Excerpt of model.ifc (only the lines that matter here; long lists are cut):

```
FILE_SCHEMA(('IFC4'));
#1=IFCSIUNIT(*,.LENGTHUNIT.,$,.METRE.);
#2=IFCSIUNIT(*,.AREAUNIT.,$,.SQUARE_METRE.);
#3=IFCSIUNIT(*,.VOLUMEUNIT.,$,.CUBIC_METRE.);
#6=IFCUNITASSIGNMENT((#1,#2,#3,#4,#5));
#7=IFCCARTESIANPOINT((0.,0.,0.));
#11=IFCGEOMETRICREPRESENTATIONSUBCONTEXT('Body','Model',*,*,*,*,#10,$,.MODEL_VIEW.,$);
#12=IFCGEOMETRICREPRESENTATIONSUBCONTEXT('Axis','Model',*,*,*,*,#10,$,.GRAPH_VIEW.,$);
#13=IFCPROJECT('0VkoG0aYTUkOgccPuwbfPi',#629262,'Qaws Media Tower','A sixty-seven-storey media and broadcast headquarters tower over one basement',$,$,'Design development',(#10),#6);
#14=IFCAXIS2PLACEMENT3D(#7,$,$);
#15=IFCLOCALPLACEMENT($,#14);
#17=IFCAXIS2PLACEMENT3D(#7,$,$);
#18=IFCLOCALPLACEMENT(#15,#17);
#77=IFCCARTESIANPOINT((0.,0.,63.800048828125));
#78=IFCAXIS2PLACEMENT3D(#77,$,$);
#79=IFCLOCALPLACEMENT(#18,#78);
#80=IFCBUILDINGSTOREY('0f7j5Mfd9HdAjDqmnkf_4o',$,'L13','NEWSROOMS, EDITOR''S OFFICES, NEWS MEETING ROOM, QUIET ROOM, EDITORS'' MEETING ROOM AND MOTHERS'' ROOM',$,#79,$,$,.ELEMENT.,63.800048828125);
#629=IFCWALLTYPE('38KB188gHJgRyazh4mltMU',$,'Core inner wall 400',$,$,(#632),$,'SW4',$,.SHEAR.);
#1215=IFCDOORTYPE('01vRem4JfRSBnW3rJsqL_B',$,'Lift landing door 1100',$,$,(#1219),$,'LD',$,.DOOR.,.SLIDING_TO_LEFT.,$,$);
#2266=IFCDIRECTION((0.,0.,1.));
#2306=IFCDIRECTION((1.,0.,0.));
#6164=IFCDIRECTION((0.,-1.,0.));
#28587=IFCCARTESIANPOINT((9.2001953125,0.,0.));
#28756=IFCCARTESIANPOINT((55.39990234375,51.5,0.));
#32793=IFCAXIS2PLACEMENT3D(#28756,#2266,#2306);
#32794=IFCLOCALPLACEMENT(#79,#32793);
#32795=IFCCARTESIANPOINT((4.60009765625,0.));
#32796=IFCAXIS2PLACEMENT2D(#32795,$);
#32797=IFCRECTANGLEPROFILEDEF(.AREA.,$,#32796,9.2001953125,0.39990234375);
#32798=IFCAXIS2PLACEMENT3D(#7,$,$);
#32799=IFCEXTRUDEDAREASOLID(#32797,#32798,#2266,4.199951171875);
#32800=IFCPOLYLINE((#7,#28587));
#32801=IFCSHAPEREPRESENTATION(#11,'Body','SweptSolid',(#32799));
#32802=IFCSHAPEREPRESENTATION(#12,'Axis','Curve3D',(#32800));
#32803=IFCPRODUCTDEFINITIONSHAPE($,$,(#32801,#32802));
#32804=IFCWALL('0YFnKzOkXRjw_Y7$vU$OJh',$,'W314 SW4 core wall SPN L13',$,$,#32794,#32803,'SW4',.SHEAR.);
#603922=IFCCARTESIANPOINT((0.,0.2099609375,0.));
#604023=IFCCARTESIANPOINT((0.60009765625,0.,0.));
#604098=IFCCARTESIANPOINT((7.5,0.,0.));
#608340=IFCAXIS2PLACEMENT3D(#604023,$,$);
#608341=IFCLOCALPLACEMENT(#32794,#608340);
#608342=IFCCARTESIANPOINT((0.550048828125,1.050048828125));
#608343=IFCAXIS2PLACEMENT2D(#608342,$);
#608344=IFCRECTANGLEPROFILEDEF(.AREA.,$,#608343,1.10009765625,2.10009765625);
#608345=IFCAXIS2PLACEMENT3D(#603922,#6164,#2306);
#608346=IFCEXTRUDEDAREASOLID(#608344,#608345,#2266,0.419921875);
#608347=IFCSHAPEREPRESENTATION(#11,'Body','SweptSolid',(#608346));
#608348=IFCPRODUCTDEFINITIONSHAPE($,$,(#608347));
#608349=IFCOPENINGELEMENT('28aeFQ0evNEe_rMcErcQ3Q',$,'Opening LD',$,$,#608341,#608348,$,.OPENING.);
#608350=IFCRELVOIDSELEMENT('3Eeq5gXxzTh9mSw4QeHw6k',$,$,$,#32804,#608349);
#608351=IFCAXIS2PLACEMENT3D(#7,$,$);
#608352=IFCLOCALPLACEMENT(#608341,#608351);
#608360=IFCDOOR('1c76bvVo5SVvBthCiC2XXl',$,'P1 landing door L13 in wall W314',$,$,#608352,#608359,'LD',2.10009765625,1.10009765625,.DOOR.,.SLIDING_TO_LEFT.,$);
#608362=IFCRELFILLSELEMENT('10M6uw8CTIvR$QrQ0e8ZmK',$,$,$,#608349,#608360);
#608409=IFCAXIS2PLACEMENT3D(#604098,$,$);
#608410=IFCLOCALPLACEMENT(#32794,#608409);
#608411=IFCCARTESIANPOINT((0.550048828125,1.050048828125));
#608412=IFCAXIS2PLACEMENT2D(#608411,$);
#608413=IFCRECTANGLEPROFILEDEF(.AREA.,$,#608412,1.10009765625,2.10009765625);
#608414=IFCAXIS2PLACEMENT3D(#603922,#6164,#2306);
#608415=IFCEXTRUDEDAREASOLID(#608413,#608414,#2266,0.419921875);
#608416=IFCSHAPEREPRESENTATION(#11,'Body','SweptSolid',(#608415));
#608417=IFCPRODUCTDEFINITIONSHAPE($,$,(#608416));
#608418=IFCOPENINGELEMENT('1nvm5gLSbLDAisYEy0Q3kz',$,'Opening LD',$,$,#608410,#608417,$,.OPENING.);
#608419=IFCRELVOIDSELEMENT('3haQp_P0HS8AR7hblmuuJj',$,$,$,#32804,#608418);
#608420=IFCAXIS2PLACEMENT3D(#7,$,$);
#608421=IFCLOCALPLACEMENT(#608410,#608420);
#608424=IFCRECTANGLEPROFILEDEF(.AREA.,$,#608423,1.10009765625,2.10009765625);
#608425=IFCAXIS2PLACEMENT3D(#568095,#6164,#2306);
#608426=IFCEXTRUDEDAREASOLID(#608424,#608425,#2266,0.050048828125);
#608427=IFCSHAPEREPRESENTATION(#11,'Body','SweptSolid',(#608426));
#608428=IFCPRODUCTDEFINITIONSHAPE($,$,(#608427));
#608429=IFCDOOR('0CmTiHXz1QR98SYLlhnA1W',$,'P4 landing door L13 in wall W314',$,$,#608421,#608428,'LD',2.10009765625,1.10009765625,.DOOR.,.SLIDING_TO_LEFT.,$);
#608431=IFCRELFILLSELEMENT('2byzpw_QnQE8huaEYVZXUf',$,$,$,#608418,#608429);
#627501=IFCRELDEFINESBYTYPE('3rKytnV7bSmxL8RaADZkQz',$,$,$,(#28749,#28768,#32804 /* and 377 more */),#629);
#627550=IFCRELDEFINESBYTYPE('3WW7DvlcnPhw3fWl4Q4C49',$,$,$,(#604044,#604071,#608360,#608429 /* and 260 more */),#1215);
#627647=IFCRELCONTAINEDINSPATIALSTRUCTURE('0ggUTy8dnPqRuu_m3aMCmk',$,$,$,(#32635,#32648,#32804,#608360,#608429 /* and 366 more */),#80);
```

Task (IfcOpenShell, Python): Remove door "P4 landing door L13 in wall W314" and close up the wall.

```python
import ifcopenshell
import ifcopenshell.api.feature
import ifcopenshell.api.root
import ifcopenshell.geom
import ifcopenshell.util.shape

model = ifcopenshell.open("model.ifc")
settings = ifcopenshell.geom.settings()


def volume(element):
    """Net volume in cubic metres, openings subtracted."""
    shape = ifcopenshell.geom.create_shape(settings, element)
    return ifcopenshell.util.shape.get_volume(shape.geometry)


door = model.by_id(608429)
opening = door.FillsVoids[0].RelatingOpeningElement
wall = opening.VoidsElements[0].RelatingBuildingElement
before = volume(wall)

ifcopenshell.api.root.remove_product(model, product=door)
ifcopenshell.api.feature.remove_feature(model, feature=opening)

after = volume(wall)

print(f"wall volume {before:.3f} -> {after:.3f} m3")

model.write("model-out.ifc")
```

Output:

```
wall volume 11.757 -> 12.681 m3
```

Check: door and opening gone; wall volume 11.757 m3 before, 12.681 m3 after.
